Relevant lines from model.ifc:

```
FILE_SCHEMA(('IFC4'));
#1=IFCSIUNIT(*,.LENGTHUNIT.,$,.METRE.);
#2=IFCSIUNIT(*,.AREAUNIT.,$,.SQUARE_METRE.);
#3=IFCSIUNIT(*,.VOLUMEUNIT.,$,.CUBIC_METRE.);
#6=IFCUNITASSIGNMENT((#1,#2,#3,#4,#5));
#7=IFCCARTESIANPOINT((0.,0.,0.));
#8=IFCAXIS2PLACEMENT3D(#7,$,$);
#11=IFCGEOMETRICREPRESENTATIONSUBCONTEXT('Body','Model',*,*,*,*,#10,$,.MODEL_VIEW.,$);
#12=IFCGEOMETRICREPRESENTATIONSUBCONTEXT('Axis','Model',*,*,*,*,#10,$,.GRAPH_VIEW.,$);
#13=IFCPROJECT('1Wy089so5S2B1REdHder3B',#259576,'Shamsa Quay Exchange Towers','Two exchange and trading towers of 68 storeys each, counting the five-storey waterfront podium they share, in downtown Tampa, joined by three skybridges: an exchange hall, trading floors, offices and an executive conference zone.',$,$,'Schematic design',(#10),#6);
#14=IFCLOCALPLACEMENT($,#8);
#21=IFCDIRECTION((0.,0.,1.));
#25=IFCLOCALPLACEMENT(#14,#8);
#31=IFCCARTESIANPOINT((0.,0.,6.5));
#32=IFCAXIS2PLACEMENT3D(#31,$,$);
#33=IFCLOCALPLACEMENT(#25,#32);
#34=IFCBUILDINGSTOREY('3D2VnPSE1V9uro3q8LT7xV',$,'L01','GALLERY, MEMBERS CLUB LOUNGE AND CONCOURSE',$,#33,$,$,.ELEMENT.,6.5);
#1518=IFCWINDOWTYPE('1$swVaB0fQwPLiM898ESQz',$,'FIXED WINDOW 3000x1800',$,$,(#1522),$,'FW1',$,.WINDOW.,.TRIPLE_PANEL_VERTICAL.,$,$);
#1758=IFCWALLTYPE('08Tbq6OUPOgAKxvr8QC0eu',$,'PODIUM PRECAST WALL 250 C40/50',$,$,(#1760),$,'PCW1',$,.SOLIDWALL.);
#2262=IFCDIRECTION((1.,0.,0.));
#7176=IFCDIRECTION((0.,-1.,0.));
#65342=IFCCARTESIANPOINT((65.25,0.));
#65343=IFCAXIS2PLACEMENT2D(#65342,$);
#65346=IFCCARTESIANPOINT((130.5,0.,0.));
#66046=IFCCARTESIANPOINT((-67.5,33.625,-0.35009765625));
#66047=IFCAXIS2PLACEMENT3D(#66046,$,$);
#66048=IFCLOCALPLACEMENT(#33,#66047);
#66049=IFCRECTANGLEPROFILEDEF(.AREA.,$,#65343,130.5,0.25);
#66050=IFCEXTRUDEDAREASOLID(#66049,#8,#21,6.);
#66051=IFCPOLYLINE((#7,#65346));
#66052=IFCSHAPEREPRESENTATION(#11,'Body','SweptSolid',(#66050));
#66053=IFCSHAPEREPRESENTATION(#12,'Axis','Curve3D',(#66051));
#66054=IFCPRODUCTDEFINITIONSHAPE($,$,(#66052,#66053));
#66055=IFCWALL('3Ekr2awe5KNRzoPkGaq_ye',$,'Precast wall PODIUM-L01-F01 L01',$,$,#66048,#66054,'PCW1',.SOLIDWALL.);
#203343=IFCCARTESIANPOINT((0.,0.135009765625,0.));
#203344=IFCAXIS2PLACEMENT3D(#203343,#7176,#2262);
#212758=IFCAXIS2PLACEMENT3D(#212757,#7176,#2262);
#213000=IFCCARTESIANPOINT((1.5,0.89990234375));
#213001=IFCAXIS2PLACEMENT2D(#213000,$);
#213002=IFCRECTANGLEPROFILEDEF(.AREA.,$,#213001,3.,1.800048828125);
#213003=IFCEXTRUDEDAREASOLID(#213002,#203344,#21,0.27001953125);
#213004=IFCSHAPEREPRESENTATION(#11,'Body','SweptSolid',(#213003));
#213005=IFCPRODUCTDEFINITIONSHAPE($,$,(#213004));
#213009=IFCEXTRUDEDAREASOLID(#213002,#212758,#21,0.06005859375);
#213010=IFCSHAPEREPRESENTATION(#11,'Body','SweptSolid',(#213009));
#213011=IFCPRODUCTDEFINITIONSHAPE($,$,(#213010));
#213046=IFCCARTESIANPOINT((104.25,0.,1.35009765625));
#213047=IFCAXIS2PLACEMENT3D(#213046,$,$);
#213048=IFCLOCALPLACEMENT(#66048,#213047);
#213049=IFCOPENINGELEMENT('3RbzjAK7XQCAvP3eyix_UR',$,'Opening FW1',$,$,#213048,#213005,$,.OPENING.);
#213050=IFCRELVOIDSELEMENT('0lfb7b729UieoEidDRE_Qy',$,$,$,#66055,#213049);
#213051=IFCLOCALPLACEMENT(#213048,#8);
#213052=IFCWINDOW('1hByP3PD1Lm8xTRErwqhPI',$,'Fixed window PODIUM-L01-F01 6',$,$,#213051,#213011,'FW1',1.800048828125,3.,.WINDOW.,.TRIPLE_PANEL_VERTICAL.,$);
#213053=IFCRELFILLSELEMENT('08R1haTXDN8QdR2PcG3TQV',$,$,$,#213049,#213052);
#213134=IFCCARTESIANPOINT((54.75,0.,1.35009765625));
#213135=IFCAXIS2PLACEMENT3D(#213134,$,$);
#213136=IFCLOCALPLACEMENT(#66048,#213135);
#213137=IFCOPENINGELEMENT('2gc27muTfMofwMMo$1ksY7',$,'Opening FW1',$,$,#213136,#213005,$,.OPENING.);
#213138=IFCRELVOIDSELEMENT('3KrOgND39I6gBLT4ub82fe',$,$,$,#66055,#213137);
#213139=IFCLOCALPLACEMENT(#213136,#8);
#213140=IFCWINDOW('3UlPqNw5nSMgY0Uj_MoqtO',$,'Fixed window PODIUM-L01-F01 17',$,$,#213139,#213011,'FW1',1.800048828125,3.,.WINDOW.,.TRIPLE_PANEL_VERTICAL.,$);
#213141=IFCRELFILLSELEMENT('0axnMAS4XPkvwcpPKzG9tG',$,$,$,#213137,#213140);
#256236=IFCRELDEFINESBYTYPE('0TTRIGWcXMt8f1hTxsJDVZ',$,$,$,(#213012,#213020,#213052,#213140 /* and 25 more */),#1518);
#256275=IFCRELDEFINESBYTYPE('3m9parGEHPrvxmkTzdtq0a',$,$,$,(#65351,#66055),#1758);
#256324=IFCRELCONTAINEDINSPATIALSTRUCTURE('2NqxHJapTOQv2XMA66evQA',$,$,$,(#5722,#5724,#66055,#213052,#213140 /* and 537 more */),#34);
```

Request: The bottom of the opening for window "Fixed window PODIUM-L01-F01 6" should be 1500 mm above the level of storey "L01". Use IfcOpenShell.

```python
import numpy as np
import ifcopenshell
import ifcopenshell.api.geometry
import ifcopenshell.geom
import ifcopenshell.util.element
import ifcopenshell.util.placement
import ifcopenshell.util.shape
import ifcopenshell.util.unit

model = ifcopenshell.open("model.ifc")
unit_scale = ifcopenshell.util.unit.calculate_unit_scale(model)

window = model.by_guid("1hByP3PD1Lm8xTRErwqhPI")
opening = window.FillsVoids[0].RelatingOpeningElement
storey = ifcopenshell.util.element.get_container(window, ifc_class="IfcBuildingStorey")
level = ifcopenshell.util.placement.get_local_placement(storey.ObjectPlacement)[2, 3]

# The opening's origin need not be at the sill, so measure its lowest point.
shape = ifcopenshell.geom.create_shape(ifcopenshell.geom.settings(), opening)
bottom = ifcopenshell.util.shape.get_shape_bottom_elevation(shape, shape.geometry) / unit_scale
dz = level + 1.5 / unit_scale - bottom

shift = np.array([0.0, 0.0, dz])
# The window is placed relative to its opening, so it follows when the opening moves.
matrix = ifcopenshell.util.placement.get_local_placement(opening.ObjectPlacement)
matrix[:3, 3] += shift
ifcopenshell.api.geometry.edit_object_placement(
    model, product=opening, matrix=matrix, is_si=False, should_transform_children=True
)

print(f"moved by {dz * unit_scale:+.3f} m")

model.write("model_v2.ifc")
```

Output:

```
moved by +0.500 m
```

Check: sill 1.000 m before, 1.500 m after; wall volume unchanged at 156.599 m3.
